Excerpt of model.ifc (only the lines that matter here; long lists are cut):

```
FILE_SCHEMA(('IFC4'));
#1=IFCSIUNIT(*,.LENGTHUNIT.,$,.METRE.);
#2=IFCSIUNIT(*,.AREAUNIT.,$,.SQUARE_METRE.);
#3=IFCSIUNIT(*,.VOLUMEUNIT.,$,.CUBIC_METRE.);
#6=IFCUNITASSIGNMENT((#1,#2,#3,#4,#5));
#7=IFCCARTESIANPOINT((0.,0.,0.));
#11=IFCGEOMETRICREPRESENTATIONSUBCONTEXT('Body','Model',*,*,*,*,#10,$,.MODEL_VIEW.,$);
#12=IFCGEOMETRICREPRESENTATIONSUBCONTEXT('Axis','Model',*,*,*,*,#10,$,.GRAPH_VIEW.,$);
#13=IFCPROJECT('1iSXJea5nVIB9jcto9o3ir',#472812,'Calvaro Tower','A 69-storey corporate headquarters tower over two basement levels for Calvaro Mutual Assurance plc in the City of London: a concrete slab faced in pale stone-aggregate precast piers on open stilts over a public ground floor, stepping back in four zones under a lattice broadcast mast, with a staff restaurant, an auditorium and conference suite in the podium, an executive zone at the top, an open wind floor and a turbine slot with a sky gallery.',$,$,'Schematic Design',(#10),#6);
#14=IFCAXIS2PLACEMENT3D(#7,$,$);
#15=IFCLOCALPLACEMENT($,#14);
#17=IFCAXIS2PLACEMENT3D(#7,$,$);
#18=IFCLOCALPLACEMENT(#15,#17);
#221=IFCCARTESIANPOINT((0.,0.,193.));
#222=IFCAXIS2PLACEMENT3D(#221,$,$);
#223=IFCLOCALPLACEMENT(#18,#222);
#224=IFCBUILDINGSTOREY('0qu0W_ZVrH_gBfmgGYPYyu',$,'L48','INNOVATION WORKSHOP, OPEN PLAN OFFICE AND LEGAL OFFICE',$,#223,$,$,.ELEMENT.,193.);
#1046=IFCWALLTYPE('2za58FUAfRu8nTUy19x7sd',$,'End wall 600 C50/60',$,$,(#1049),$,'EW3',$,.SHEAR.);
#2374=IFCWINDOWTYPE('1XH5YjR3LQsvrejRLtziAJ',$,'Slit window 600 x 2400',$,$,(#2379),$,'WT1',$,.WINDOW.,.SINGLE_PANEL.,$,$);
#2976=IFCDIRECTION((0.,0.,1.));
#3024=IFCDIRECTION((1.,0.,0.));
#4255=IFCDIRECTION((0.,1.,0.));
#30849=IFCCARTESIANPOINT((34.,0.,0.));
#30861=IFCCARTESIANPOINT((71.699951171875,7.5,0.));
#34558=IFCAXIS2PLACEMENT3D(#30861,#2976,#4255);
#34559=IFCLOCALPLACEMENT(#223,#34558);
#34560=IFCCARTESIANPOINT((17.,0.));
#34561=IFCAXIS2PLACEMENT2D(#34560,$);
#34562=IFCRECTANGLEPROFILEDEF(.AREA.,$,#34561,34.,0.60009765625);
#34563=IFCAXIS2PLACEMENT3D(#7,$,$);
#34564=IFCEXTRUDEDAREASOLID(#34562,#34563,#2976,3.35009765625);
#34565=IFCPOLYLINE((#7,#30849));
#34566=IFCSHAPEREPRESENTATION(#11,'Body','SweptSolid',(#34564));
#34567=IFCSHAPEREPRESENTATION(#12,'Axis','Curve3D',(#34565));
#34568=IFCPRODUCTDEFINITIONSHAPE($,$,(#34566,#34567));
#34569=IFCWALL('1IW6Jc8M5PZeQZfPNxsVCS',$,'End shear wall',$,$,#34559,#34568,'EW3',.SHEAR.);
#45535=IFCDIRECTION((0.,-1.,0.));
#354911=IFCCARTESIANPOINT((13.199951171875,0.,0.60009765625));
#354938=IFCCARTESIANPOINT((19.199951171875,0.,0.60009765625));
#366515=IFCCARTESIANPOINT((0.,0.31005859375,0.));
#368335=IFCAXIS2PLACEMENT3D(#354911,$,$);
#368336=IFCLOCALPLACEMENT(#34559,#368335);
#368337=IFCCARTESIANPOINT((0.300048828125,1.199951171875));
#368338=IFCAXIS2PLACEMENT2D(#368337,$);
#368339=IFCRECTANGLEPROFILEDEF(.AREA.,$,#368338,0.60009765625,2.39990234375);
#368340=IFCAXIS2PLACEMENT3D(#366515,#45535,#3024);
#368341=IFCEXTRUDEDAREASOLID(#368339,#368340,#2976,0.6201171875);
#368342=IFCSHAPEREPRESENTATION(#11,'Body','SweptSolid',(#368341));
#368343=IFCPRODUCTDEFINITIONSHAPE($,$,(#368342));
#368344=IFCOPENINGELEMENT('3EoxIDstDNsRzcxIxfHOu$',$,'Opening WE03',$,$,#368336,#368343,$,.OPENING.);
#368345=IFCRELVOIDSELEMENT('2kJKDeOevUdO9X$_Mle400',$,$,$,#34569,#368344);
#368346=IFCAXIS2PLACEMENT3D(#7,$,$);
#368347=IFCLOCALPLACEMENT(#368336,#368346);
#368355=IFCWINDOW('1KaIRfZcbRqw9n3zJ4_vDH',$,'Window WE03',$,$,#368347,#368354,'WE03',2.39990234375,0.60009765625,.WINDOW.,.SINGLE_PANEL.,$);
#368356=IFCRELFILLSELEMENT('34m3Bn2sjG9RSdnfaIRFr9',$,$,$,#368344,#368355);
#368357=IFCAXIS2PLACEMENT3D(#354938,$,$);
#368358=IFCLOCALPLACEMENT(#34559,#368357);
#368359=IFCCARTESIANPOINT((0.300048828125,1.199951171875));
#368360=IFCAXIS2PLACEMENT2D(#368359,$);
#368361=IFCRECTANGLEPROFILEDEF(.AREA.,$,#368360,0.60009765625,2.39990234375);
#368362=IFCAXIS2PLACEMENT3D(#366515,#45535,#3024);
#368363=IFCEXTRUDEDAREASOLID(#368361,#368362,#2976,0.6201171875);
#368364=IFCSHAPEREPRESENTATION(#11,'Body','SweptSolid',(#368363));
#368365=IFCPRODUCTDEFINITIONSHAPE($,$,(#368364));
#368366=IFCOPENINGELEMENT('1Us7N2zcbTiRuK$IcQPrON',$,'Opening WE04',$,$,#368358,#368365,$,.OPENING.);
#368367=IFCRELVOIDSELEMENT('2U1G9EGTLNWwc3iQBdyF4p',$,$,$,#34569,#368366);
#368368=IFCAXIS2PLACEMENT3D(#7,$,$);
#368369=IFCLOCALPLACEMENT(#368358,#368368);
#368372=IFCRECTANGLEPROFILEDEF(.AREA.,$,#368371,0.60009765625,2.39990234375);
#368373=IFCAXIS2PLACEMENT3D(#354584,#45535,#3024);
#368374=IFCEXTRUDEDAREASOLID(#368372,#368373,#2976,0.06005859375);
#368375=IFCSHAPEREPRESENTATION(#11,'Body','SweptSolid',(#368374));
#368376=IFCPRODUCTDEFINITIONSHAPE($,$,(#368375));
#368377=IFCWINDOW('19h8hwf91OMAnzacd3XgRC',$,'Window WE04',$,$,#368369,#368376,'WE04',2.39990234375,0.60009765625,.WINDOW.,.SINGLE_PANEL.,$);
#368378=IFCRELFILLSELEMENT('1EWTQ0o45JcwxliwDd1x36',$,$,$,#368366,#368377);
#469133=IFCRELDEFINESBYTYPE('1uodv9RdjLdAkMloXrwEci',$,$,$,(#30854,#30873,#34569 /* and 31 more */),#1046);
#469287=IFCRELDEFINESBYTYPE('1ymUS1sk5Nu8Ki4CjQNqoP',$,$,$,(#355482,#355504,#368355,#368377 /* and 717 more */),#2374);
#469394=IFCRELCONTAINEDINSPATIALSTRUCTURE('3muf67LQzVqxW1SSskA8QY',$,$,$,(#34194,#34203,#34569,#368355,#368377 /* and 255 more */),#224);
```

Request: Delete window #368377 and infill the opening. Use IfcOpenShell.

```python
import ifcopenshell
import ifcopenshell.api.feature
import ifcopenshell.api.root
import ifcopenshell.geom
import ifcopenshell.util.shape

model = ifcopenshell.open("model.ifc")
settings = ifcopenshell.geom.settings()


def volume(element):
    """Net volume in cubic metres, openings subtracted."""
    shape = ifcopenshell.geom.create_shape(settings, element)
    return ifcopenshell.util.shape.get_volume(shape.geometry)


window = model.by_guid("19h8hwf91OMAnzacd3XgRC")
opening = window.FillsVoids[0].RelatingOpeningElement
wall = opening.VoidsElements[0].RelatingBuildingElement
before = volume(wall)

ifcopenshell.api.root.remove_product(model, product=window)
ifcopenshell.api.feature.remove_feature(model, feature=opening)

after = volume(wall)

print(f"wall volume {before:.3f} -> {after:.3f} m3")

model.write("model_v2.ifc")
```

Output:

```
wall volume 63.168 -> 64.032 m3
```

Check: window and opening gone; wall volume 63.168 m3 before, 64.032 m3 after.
